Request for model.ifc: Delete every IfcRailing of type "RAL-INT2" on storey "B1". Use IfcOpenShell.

First a look at what the model holds.

```python
import ifcopenshell
import ifcopenshell.util.element

model = ifcopenshell.open("model.ifc")
print(model.schema)
storey = next(s for s in model.by_type("IfcBuildingStorey") if s.Name == "B1")
railings = [e for e in ifcopenshell.util.element.get_decomposition(storey) if e.is_a("IfcRailing")]
seen = {}
for e in railings:
    element_type = ifcopenshell.util.element.get_type(e)
    name = element_type.Name if element_type not in (None, e) else None
    seen[name] = seen.get(name, 0) + 1
for name, count in sorted(seen.items(), key=str):
    print(count, "x", name)
```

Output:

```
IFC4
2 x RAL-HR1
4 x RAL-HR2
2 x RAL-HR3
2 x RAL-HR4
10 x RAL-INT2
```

```python
import ifcopenshell
import ifcopenshell.api.root
import ifcopenshell.util.element

model = ifcopenshell.open("model.ifc")

storey = next(s for s in model.by_type("IfcBuildingStorey") if s.Name == "B1")
railings = [e for e in ifcopenshell.util.element.get_decomposition(storey) if e.is_a("IfcRailing")]
targets = [e for e in railings if (t := ifcopenshell.util.element.get_type(e)) not in (None, e) and t.Name == "RAL-INT2"]

for e in targets:
    ifcopenshell.api.root.remove_product(model, product=e)
print(len(targets), "removed")

model.write("model-out.ifc")
```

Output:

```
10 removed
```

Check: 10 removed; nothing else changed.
